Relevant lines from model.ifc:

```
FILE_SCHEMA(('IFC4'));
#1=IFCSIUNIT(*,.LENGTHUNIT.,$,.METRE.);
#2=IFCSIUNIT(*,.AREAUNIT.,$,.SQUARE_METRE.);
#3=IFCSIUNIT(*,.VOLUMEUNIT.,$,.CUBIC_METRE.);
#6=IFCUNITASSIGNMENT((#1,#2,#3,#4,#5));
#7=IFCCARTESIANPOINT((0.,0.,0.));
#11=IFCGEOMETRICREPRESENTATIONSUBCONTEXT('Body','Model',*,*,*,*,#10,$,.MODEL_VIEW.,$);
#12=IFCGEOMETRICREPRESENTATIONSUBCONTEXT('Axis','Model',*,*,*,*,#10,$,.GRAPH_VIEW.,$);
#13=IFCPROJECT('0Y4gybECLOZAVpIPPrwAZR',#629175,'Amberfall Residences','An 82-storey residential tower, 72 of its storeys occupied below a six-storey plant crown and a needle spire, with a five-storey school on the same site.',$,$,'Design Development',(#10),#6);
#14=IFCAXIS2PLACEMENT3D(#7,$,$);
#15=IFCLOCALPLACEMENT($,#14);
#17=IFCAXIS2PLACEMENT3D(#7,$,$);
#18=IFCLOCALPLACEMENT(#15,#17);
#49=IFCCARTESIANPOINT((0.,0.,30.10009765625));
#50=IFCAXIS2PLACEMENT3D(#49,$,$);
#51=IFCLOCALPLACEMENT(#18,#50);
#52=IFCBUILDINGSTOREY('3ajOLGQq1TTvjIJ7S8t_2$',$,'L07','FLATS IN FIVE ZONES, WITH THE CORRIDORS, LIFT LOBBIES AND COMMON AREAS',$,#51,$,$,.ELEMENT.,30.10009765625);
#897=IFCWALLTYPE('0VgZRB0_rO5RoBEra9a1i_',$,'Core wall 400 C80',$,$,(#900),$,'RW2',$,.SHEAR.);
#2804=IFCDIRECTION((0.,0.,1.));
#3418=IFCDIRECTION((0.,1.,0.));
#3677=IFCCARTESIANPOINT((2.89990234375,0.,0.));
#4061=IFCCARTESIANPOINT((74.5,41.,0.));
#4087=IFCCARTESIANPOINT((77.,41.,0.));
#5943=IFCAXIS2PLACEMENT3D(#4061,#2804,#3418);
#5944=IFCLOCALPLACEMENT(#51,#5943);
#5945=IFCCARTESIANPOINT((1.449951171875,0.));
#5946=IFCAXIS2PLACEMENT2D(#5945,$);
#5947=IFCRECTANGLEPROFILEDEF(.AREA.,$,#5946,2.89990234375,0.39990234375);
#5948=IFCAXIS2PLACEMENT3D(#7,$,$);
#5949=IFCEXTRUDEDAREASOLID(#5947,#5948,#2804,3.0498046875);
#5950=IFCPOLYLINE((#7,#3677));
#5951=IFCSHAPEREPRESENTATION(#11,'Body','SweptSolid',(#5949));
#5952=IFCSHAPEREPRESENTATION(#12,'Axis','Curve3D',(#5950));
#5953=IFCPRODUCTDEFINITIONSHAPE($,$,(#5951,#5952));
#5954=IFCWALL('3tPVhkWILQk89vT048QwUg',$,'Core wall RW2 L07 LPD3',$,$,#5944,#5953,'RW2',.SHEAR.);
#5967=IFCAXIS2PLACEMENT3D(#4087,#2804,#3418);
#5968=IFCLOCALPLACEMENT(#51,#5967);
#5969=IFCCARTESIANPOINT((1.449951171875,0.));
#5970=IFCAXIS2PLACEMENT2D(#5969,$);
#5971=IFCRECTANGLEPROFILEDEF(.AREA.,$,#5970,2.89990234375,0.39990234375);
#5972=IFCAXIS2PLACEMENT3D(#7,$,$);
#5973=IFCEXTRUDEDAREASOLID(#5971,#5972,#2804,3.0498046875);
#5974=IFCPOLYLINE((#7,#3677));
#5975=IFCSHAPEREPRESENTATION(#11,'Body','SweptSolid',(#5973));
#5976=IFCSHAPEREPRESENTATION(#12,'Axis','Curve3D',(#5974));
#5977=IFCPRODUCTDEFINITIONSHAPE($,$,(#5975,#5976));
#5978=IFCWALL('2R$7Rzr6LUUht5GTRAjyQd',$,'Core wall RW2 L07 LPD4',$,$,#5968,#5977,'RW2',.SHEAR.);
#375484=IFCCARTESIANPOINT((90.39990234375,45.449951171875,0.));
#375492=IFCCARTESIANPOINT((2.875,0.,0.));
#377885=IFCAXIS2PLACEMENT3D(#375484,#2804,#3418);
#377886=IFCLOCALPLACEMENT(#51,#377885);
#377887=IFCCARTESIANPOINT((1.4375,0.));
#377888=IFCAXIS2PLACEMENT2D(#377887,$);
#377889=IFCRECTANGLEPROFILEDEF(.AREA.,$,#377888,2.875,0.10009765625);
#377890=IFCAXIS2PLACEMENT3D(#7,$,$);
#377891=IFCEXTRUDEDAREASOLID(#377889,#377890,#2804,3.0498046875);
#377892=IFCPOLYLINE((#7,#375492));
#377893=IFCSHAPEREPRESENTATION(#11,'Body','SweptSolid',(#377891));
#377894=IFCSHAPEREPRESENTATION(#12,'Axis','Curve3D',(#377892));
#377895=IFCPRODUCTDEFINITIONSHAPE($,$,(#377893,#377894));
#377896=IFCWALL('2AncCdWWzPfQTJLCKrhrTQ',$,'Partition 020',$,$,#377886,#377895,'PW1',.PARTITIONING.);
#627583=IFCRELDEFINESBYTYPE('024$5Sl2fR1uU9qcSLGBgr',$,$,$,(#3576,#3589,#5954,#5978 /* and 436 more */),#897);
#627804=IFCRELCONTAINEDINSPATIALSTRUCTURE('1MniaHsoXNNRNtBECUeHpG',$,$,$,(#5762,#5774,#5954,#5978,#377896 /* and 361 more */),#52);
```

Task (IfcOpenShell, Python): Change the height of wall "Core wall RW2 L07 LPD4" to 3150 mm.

```python
import ifcopenshell
import ifcopenshell.geom
import ifcopenshell.util.representation
import ifcopenshell.util.shape

model = ifcopenshell.open("model.ifc")
settings = ifcopenshell.geom.settings()


def volume(element):
    """Net volume in cubic metres, openings subtracted."""
    shape = ifcopenshell.geom.create_shape(settings, element)
    return ifcopenshell.util.shape.get_volume(shape.geometry)


wall = model.by_guid("2R$7Rzr6LUUht5GTRAjyQd")
before = volume(wall)

body = ifcopenshell.util.representation.get_representation(wall, "Model", "Body")
solid = body.Items[0]
old_height = solid.Depth
solid.Depth = 3.15
after = volume(wall)

print(f"height {old_height:g} -> {solid.Depth:g}, volume {before:.3f} -> {after:.3f} m3")

model.write("model_updated.ifc")
```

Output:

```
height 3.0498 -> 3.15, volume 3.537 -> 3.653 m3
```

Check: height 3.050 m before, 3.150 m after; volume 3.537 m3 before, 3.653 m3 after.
